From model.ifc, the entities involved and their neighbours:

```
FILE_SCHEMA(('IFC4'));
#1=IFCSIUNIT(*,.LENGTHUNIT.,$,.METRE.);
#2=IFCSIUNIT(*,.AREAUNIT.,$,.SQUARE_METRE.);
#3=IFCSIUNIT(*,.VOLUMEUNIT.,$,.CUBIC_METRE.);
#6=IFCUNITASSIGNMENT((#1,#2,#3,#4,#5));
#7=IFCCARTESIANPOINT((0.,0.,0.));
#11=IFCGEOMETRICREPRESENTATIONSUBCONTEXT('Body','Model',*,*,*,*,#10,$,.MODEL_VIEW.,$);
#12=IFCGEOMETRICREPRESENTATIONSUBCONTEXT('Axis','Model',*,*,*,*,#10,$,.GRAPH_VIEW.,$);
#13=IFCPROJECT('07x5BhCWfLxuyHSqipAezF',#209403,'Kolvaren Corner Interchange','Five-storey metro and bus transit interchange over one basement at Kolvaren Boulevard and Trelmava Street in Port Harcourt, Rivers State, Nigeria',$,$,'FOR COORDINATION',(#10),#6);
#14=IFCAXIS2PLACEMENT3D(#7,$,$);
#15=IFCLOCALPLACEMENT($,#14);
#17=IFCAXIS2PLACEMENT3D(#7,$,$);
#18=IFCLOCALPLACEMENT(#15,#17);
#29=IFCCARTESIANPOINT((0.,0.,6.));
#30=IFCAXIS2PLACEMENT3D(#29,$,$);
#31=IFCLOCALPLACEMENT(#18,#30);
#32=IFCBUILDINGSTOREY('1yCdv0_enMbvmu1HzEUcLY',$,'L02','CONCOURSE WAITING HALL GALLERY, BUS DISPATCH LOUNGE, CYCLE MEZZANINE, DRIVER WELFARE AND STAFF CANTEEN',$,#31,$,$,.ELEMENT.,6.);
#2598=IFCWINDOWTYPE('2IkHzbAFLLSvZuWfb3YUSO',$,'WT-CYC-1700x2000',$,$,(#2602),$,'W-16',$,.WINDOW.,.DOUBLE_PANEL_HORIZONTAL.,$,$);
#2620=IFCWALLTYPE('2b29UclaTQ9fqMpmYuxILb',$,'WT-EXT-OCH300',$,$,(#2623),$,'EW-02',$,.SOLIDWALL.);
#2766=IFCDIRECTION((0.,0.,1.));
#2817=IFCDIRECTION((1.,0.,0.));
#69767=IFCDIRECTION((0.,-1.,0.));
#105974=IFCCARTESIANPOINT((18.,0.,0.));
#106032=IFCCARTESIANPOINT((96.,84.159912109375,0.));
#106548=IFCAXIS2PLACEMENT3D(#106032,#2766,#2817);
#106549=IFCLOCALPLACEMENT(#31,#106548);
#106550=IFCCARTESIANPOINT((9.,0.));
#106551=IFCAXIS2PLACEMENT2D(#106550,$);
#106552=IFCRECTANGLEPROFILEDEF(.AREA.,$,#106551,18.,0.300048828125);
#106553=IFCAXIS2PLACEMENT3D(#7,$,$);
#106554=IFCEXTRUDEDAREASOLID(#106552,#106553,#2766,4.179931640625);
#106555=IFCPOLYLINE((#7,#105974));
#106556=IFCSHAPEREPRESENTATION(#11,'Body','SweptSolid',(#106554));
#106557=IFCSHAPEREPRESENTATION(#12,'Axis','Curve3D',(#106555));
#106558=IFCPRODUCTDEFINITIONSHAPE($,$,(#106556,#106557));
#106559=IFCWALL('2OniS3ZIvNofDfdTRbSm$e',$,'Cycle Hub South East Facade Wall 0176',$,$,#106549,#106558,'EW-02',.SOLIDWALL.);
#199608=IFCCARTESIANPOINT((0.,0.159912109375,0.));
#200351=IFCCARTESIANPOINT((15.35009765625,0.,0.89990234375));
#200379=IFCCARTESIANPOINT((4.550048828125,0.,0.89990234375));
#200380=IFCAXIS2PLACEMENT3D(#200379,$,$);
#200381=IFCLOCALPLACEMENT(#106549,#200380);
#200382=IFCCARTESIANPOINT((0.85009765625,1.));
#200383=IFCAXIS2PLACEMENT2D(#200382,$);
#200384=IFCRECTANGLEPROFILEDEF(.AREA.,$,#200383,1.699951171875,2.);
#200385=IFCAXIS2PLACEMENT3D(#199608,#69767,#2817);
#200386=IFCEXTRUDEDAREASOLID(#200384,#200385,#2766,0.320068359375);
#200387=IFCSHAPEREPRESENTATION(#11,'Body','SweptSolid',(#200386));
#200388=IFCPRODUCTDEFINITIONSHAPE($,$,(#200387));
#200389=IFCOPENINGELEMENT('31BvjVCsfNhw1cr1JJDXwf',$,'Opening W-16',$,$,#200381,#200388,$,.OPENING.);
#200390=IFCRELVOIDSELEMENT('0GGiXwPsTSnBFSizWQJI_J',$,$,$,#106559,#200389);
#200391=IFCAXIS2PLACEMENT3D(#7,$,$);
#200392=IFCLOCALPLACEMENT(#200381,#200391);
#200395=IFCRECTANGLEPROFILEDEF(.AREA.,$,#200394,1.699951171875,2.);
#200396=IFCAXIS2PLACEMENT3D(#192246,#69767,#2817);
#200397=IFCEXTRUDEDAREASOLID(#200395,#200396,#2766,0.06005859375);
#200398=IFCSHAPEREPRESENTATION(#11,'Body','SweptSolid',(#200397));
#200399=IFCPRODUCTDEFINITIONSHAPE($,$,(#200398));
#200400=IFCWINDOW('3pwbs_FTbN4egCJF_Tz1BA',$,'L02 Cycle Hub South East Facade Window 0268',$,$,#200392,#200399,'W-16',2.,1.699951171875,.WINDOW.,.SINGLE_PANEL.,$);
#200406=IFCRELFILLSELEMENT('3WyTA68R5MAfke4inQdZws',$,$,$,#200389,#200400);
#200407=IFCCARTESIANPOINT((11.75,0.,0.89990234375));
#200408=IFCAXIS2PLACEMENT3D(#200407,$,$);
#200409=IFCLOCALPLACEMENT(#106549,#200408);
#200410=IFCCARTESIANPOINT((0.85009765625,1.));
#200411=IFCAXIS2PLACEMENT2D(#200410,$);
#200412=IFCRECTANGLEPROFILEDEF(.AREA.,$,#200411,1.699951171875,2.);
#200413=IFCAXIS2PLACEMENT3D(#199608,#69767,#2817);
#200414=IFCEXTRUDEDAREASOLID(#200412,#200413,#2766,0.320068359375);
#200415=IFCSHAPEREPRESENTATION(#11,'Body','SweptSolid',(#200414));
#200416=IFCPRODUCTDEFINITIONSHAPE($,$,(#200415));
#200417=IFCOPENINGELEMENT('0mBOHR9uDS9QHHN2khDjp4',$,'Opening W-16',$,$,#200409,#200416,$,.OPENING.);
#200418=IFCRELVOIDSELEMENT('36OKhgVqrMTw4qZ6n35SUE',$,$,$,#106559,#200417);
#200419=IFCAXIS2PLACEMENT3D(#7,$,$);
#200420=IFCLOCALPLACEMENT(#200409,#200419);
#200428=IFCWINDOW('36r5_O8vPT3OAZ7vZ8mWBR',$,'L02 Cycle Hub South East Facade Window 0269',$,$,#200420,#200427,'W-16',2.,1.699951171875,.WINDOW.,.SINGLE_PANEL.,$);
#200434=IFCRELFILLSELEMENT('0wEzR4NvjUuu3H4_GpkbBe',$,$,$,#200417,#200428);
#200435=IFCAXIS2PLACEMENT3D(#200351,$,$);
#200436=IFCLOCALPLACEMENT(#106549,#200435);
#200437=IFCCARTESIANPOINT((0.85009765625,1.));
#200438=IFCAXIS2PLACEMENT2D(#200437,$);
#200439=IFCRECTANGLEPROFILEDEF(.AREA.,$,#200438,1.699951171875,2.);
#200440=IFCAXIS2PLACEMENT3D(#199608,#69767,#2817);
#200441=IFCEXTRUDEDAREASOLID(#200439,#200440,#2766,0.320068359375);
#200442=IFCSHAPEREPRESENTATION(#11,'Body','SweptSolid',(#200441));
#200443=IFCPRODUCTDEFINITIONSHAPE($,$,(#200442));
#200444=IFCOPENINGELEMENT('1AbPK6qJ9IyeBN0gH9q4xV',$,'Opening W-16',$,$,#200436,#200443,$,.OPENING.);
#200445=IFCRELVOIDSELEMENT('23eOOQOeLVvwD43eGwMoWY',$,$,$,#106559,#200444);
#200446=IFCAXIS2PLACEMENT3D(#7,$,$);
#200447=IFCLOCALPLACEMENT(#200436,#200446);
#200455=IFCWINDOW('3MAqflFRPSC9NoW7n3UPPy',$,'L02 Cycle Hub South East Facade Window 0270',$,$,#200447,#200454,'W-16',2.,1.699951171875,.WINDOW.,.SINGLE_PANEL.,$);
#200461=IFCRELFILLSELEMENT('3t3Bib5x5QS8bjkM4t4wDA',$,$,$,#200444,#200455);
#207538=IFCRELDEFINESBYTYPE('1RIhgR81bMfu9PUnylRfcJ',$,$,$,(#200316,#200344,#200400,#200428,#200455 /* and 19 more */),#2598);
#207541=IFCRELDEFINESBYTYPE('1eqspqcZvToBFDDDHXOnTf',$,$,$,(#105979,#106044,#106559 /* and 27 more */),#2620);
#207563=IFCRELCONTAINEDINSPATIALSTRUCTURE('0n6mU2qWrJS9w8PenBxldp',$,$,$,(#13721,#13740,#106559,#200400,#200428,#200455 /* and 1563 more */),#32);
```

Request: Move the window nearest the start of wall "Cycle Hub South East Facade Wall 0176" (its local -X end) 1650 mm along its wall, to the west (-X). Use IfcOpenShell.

```python
import ifcopenshell
import ifcopenshell.api.geometry
import ifcopenshell.util.placement
import ifcopenshell.util.unit

model = ifcopenshell.open("model.ifc")
unit_scale = ifcopenshell.util.unit.calculate_unit_scale(model)

window = model.by_id(200400)
opening = window.FillsVoids[0].RelatingOpeningElement
wall = opening.VoidsElements[0].RelatingBuildingElement

wall_matrix = ifcopenshell.util.placement.get_local_placement(wall.ObjectPlacement)
shift = wall_matrix[:3, 0] * -1.65 / unit_scale
before = ifcopenshell.util.placement.get_local_placement(window.ObjectPlacement)[:3, 3].copy()

# The window is placed relative to its opening, so it follows when the opening moves.
matrix = ifcopenshell.util.placement.get_local_placement(opening.ObjectPlacement)
matrix[:3, 3] += shift
ifcopenshell.api.geometry.edit_object_placement(
    model, product=opening, matrix=matrix, is_si=False, should_transform_children=True
)

after = ifcopenshell.util.placement.get_local_placement(window.ObjectPlacement)[:3, 3]
print("window moved by", (after - before).round(3) + 0.0)

model.write("model_rev.ifc")
```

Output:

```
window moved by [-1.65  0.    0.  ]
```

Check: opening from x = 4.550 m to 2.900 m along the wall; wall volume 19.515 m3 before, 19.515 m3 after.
